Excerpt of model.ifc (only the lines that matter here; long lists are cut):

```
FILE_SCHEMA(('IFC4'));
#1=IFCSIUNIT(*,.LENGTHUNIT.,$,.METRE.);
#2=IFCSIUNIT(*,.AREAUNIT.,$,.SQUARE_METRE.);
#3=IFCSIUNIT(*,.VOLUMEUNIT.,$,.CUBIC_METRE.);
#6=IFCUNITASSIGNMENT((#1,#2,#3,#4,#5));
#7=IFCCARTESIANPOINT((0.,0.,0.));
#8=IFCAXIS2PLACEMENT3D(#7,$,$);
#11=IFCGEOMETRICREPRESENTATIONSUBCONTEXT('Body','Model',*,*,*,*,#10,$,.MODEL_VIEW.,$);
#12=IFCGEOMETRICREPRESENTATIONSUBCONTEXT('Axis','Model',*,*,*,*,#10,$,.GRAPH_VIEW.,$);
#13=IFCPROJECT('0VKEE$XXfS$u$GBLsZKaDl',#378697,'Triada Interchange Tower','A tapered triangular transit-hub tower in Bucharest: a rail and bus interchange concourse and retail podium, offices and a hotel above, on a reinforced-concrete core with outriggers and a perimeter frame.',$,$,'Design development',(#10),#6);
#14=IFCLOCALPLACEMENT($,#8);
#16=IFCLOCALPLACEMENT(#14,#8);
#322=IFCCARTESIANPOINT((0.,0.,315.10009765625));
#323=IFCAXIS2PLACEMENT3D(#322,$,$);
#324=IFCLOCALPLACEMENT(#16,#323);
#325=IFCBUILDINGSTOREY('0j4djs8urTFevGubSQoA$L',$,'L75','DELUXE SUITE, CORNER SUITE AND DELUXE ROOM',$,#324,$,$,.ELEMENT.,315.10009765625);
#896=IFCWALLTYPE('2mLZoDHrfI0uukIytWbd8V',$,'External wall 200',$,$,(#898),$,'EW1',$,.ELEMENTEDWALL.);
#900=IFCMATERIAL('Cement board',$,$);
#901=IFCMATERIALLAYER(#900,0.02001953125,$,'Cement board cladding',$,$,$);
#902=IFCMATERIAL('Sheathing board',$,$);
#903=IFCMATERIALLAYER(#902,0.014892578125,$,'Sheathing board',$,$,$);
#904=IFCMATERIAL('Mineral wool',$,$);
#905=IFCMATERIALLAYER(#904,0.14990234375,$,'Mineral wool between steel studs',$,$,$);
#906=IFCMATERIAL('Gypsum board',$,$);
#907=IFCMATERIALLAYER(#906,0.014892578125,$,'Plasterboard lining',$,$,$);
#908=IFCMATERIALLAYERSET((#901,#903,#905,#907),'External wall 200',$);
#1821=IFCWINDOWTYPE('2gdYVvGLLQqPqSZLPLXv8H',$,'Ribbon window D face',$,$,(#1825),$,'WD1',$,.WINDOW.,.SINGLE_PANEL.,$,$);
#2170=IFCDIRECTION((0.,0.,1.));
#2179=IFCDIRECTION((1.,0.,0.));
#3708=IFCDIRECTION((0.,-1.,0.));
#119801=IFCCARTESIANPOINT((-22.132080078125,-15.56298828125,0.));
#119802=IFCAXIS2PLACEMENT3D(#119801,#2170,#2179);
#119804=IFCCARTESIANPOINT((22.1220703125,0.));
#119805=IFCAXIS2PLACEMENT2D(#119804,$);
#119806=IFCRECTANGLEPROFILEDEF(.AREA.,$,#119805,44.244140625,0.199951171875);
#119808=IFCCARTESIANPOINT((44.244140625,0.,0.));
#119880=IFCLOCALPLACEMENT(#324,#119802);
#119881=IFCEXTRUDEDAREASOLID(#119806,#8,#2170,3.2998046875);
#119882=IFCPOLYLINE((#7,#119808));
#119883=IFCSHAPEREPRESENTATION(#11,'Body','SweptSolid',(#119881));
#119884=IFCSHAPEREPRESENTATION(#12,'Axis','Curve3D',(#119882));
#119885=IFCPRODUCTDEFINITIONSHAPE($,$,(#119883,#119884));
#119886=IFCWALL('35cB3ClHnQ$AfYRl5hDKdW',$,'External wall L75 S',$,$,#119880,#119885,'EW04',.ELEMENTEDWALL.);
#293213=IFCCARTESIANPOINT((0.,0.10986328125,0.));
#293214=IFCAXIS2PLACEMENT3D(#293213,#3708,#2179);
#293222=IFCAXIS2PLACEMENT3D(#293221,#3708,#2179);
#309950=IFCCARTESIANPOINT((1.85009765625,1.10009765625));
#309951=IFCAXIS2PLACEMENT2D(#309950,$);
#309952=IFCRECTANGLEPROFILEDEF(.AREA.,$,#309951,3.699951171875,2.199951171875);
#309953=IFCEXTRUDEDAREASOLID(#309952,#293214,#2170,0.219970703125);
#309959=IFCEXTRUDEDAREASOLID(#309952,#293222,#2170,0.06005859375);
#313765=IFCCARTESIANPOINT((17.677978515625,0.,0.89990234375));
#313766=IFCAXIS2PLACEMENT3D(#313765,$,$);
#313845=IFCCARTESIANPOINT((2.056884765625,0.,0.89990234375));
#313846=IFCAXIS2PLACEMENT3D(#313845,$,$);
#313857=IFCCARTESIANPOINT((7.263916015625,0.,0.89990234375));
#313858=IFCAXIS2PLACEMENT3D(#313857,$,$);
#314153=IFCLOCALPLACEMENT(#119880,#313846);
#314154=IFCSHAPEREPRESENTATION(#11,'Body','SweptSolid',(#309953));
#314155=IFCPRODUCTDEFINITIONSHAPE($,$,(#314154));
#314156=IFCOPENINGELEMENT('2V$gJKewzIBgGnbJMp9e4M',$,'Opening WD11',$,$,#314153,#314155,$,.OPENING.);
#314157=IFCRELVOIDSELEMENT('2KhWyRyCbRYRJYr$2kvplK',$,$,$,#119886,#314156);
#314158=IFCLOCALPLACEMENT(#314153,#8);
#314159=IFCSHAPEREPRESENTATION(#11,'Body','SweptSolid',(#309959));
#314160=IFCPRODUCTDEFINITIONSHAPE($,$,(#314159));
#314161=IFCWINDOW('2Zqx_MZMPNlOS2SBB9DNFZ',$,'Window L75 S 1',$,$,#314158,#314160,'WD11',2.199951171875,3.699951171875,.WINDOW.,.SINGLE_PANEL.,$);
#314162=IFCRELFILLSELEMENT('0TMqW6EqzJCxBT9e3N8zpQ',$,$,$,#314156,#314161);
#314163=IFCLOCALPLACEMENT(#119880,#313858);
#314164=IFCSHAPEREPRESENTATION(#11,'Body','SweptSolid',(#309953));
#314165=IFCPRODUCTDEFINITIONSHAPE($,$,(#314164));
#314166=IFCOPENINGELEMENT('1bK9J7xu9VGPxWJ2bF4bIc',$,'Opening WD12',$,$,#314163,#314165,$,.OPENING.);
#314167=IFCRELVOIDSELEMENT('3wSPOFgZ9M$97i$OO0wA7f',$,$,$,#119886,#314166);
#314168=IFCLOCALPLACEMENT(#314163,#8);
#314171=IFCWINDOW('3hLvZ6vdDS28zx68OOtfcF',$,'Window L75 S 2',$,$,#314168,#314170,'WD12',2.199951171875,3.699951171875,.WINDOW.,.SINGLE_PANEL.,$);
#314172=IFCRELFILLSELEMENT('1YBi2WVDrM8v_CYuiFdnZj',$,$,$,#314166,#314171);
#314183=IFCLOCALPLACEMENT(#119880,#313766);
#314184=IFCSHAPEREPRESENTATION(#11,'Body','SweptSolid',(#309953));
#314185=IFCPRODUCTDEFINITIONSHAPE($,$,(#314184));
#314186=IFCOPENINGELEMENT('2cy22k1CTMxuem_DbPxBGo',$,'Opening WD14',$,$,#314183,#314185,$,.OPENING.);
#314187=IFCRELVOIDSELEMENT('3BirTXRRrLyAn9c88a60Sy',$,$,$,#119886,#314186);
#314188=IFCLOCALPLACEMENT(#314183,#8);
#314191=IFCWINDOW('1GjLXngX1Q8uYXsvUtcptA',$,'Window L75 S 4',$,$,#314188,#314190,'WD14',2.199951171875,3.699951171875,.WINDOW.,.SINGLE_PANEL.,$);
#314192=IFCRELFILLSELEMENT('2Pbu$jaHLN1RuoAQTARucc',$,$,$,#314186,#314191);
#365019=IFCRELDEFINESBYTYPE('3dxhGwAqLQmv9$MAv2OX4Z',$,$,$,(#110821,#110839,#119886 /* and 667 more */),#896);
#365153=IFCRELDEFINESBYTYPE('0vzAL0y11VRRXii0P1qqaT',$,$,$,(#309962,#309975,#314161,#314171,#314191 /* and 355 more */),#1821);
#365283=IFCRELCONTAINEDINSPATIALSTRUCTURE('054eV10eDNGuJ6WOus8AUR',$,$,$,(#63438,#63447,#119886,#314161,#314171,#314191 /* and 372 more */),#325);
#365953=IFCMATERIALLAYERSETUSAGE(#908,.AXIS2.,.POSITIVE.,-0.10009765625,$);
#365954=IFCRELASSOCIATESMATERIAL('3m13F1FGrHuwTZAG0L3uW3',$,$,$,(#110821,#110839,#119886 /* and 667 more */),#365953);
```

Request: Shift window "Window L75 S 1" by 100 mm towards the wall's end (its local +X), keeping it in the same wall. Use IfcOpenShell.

```python
import ifcopenshell
import ifcopenshell.api.geometry
import ifcopenshell.util.placement
import ifcopenshell.util.unit

model = ifcopenshell.open("model.ifc")
unit_scale = ifcopenshell.util.unit.calculate_unit_scale(model)

window = model.by_guid("2Zqx_MZMPNlOS2SBB9DNFZ")
opening = window.FillsVoids[0].RelatingOpeningElement
wall = opening.VoidsElements[0].RelatingBuildingElement

wall_matrix = ifcopenshell.util.placement.get_local_placement(wall.ObjectPlacement)
shift = wall_matrix[:3, 0] * 0.1 / unit_scale
before = ifcopenshell.util.placement.get_local_placement(window.ObjectPlacement)[:3, 3].copy()

# The window is placed relative to its opening, so it follows when the opening moves.
matrix = ifcopenshell.util.placement.get_local_placement(opening.ObjectPlacement)
matrix[:3, 3] += shift
ifcopenshell.api.geometry.edit_object_placement(
    model, product=opening, matrix=matrix, is_si=False, should_transform_children=True
)

after = ifcopenshell.util.placement.get_local_placement(window.ObjectPlacement)[:3, 3]
print("window moved by", (after - before).round(3) + 0.0)

model.write("model_v2.ifc")
```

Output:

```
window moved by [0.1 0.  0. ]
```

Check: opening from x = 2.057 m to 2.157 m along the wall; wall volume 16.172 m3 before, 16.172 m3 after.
